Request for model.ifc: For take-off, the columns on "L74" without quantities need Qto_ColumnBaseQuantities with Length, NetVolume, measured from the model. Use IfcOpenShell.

First a look at what the model holds.

```python
import ifcopenshell
import ifcopenshell.util.element
import ifcopenshell.util.unit

model = ifcopenshell.open("model.ifc")
print(model.schema)
for unit_type in ("LENGTHUNIT", "AREAUNIT", "VOLUMEUNIT"):
    print(unit_type, ifcopenshell.util.unit.calculate_unit_scale(model, unit_type))
storey = next(s for s in model.by_type("IfcBuildingStorey") if s.Name == "L74")
columns = [e for e in ifcopenshell.util.element.get_decomposition(storey) if e.is_a("IfcColumn")]
for e in sorted(columns, key=lambda e: e.id()):
    print(e.id(), e.is_a(), e.Name, list(ifcopenshell.util.element.get_psets(e, qtos_only=True)), sep=" | ")
```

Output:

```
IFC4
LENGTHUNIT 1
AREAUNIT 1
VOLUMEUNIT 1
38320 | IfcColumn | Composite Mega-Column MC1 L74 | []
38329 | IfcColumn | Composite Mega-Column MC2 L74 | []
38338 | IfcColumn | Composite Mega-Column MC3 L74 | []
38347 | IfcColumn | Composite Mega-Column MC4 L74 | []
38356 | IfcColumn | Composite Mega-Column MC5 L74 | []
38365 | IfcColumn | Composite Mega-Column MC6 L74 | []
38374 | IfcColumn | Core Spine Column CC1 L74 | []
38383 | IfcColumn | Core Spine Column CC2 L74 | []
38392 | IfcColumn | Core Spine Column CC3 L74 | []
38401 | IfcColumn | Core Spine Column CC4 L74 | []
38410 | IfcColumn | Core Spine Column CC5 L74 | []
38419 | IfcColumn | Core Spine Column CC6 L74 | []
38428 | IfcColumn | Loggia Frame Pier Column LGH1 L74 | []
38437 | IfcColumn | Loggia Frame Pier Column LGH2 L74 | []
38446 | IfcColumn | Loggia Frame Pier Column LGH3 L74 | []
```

```python
import ifcopenshell
import ifcopenshell.api.pset
import ifcopenshell.geom
import ifcopenshell.util.element
import ifcopenshell.util.shape
import ifcopenshell.util.unit

model = ifcopenshell.open("model.ifc")
unit_scale = ifcopenshell.util.unit.calculate_unit_scale(model)
volume_scale = ifcopenshell.util.unit.calculate_unit_scale(model, "VOLUMEUNIT")
settings = ifcopenshell.geom.settings()

storey = next(s for s in model.by_type("IfcBuildingStorey") if s.Name == "L74")
columns = [e for e in ifcopenshell.util.element.get_decomposition(storey) if e.is_a("IfcColumn")]

for e in sorted(columns, key=lambda e: e.id()):
    if ifcopenshell.util.element.get_psets(e, qtos_only=True, should_inherit=False):
        continue
    # Geometry comes back in metres, in the element's own axes.
    shape = ifcopenshell.geom.create_shape(settings, e)
    values = {
        "Length": ifcopenshell.util.shape.get_z(shape.geometry) / unit_scale,
        "NetVolume": ifcopenshell.util.shape.get_volume(shape.geometry) / volume_scale,
    }
    qto = ifcopenshell.api.pset.add_qto(model, product=e, name="Qto_ColumnBaseQuantities")
    ifcopenshell.api.pset.edit_qto(model, qto=qto, properties=values)
    print(e.id(), {k: round(v, 3) for k, v in values.items()})

model.write("model_v2.ifc")
```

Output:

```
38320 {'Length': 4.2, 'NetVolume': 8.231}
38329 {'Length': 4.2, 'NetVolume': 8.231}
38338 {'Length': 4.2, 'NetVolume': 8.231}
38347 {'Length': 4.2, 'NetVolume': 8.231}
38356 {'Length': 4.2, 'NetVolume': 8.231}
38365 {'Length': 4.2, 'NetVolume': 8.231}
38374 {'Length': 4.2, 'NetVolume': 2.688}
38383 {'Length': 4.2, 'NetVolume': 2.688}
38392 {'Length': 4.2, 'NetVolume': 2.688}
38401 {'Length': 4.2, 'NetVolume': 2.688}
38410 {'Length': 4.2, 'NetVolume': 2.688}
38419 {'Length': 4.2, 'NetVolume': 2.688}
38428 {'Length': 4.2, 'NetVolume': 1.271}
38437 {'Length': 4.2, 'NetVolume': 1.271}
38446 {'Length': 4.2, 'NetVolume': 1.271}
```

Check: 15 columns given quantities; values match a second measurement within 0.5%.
